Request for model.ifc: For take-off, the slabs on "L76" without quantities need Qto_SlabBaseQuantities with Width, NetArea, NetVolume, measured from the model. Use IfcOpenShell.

First a look at what the model holds.

```python
import ifcopenshell
import ifcopenshell.util.element
import ifcopenshell.util.unit

model = ifcopenshell.open("model.ifc")
print(model.schema)
for unit_type in ("LENGTHUNIT", "AREAUNIT", "VOLUMEUNIT"):
    print(unit_type, ifcopenshell.util.unit.calculate_unit_scale(model, unit_type))
storey = next(s for s in model.by_type("IfcBuildingStorey") if s.Name == "L76")
slabs = [e for e in ifcopenshell.util.element.get_decomposition(storey) if e.is_a("IfcSlab")]
for e in sorted(slabs, key=lambda e: e.id()):
    print(e.id(), e.is_a(), e.Name, list(ifcopenshell.util.element.get_psets(e, qtos_only=True)), sep=" | ")
```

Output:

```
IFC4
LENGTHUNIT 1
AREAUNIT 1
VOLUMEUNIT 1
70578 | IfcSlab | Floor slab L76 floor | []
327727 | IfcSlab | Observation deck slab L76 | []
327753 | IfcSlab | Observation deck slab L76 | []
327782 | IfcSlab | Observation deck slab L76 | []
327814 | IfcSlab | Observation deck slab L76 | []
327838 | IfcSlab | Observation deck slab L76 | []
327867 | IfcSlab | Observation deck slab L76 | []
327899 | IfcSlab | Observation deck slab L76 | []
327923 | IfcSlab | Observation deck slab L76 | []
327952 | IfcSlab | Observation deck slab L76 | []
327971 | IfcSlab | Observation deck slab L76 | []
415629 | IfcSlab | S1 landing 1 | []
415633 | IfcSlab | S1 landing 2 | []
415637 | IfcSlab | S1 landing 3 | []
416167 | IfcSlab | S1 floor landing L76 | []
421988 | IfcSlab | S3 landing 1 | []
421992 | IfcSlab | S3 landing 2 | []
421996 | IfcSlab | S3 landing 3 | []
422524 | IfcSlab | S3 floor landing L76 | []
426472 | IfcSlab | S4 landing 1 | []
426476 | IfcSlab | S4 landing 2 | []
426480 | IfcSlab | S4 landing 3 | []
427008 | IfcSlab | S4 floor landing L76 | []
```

```python
import ifcopenshell
import ifcopenshell.api.pset
import ifcopenshell.geom
import ifcopenshell.util.element
import ifcopenshell.util.shape
import ifcopenshell.util.unit

model = ifcopenshell.open("model.ifc")
unit_scale = ifcopenshell.util.unit.calculate_unit_scale(model)
area_scale = ifcopenshell.util.unit.calculate_unit_scale(model, "AREAUNIT")
volume_scale = ifcopenshell.util.unit.calculate_unit_scale(model, "VOLUMEUNIT")
settings = ifcopenshell.geom.settings()

storey = next(s for s in model.by_type("IfcBuildingStorey") if s.Name == "L76")
slabs = [e for e in ifcopenshell.util.element.get_decomposition(storey) if e.is_a("IfcSlab")]

for e in sorted(slabs, key=lambda e: e.id()):
    if ifcopenshell.util.element.get_psets(e, qtos_only=True, should_inherit=False):
        continue
    # Geometry comes back in metres, in the element's own axes.
    shape = ifcopenshell.geom.create_shape(settings, e)
    values = {
        "Width": ifcopenshell.util.shape.get_z(shape.geometry) / unit_scale,
        "NetArea": ifcopenshell.util.shape.get_footprint_area(shape.geometry) / area_scale,
        "NetVolume": ifcopenshell.util.shape.get_volume(shape.geometry) / volume_scale,
    }
    qto = ifcopenshell.api.pset.add_qto(model, product=e, name="Qto_SlabBaseQuantities")
    ifcopenshell.api.pset.edit_qto(model, qto=qto, properties=values)
    print(e.id(), {k: round(v, 3) for k, v in values.items()})

model.write("model_updated.ifc")
```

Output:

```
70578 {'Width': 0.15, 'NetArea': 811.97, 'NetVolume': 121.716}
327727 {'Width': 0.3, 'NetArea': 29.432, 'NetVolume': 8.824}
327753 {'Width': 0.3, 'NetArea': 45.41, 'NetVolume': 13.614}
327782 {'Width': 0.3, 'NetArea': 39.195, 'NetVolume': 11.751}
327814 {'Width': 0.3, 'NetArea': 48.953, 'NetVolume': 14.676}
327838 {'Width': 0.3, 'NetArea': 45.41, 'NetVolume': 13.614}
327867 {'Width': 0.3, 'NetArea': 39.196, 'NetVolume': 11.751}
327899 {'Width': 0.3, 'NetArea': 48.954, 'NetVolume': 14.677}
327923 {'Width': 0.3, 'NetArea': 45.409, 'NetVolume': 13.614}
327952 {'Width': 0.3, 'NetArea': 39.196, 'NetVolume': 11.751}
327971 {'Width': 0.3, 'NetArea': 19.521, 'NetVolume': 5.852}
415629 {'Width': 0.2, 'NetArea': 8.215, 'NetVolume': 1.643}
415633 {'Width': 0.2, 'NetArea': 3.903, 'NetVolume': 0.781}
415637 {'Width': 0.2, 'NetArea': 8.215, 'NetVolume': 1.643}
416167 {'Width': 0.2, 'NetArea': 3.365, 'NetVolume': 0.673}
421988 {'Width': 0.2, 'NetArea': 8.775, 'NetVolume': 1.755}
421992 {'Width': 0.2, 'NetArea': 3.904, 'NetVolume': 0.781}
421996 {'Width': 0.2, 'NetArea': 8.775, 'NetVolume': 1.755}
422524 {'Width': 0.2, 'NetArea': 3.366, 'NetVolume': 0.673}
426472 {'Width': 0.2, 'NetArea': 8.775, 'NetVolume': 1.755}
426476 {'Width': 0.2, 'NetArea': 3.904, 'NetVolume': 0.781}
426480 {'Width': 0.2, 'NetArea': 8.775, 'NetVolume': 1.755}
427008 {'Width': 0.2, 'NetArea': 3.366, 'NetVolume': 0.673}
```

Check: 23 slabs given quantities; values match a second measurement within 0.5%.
